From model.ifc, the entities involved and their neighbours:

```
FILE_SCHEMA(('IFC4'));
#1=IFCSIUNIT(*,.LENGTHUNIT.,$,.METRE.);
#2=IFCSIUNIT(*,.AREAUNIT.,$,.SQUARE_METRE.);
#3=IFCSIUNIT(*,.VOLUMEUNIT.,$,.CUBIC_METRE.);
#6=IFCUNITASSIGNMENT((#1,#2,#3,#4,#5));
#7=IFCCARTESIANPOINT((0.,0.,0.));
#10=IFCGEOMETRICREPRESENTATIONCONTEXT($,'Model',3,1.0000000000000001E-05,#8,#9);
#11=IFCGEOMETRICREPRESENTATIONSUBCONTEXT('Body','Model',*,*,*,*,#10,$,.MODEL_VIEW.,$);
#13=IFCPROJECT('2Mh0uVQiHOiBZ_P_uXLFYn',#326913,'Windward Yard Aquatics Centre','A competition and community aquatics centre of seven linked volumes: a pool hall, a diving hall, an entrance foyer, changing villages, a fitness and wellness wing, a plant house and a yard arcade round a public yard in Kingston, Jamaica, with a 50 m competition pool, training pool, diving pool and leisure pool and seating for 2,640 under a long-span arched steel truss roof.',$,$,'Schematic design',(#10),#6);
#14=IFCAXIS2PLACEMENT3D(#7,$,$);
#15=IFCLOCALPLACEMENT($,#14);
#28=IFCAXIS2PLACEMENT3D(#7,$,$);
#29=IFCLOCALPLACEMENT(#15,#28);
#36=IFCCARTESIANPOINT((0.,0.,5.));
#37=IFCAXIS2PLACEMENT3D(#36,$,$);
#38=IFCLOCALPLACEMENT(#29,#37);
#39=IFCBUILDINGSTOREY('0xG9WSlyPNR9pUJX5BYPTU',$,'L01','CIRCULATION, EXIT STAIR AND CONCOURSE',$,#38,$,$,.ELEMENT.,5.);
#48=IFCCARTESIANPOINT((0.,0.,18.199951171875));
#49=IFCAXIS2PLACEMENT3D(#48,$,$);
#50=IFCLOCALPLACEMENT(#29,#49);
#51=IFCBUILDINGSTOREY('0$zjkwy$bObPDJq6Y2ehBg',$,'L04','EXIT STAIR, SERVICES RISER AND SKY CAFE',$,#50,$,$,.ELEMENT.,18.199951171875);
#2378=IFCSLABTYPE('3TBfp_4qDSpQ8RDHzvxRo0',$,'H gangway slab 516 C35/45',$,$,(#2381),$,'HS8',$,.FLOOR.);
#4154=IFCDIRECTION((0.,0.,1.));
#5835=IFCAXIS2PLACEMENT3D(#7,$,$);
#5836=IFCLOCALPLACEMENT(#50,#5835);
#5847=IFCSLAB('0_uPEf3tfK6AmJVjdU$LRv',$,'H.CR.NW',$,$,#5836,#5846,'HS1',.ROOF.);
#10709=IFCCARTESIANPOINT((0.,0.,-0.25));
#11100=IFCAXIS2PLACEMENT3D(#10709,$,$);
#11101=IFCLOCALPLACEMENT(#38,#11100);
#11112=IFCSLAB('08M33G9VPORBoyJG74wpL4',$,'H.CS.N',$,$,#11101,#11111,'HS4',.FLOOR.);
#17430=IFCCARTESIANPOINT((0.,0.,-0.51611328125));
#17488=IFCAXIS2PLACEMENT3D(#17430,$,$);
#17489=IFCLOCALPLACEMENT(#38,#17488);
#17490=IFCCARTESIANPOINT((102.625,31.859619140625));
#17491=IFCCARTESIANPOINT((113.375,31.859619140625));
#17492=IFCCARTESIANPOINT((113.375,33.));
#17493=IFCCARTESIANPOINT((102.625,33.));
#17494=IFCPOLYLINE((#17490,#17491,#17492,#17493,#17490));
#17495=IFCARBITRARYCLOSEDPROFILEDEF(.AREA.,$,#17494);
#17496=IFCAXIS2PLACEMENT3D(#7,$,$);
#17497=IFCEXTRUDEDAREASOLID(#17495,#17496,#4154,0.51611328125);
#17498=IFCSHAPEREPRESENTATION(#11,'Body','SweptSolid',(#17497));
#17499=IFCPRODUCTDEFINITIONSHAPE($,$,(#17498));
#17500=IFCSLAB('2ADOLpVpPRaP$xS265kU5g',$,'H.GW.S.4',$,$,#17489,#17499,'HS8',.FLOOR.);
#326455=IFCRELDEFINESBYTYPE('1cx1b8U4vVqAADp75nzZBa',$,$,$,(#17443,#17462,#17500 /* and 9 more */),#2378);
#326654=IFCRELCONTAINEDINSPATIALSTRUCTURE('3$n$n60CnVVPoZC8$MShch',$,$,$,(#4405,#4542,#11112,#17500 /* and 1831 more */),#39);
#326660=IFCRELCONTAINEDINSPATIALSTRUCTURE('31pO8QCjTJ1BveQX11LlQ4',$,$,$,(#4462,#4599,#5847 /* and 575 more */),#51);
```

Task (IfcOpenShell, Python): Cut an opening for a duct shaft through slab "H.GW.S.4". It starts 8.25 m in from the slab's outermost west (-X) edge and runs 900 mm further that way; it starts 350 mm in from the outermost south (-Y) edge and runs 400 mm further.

```python
import numpy as np
import ifcopenshell
import ifcopenshell.api.feature
import ifcopenshell.api.geometry
import ifcopenshell.api.root
import ifcopenshell.geom
import ifcopenshell.util.placement
import ifcopenshell.util.representation
import ifcopenshell.util.shape
import ifcopenshell.util.unit

model = ifcopenshell.open("model.ifc")
unit_scale = ifcopenshell.util.unit.calculate_unit_scale(model)
settings = ifcopenshell.geom.settings()


def volume(element):
    """Net volume in cubic metres, openings subtracted."""
    shape = ifcopenshell.geom.create_shape(settings, element)
    return ifcopenshell.util.shape.get_volume(shape.geometry)


slab = model.by_id(17500)
before = volume(slab)

# Extent in the slab's own axes, in metres. The edges named are its -X and -Y sides.
slab_shape = ifcopenshell.geom.create_shape(settings, slab)
vertices = ifcopenshell.util.shape.get_vertices(slab_shape.geometry)
x_min, y_min, bottom = vertices.min(axis=0)
top = vertices[:, 2].max()

opening = ifcopenshell.api.root.create_entity(model, ifc_class="IfcOpeningElement", name="Duct shaft opening", predefined_type="OPENING")
context = ifcopenshell.util.representation.get_context(model, "Model", "Body", "MODEL_VIEW")
width, depth = 0.9, 0.4
outline = [(0.0, 0.0), (width, 0.0), (width, depth), (0.0, depth), (0.0, 0.0)]
# Overshoot both faces by 50 mm so the cut is clean.
shape = ifcopenshell.api.geometry.add_slab_representation(
    model, context=context, depth=top - bottom + 0.1, polyline=outline
)
ifcopenshell.api.geometry.assign_representation(model, product=opening, representation=shape)

matrix = ifcopenshell.util.placement.get_local_placement(slab.ObjectPlacement)
matrix[:, 3] = matrix @ np.append(np.array([x_min + 8.25, y_min + 0.35, bottom - 0.05]) / unit_scale, 1.0)
ifcopenshell.api.geometry.edit_object_placement(model, product=opening, matrix=matrix, is_si=False)
ifcopenshell.api.feature.add_feature(model, feature=opening, element=slab)

after = volume(slab)

print(f"slab volume {before:.3f} -> {after:.3f} m3")

model.write("model-out.ifc")
```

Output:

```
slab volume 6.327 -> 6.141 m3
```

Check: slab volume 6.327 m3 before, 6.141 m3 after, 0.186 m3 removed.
